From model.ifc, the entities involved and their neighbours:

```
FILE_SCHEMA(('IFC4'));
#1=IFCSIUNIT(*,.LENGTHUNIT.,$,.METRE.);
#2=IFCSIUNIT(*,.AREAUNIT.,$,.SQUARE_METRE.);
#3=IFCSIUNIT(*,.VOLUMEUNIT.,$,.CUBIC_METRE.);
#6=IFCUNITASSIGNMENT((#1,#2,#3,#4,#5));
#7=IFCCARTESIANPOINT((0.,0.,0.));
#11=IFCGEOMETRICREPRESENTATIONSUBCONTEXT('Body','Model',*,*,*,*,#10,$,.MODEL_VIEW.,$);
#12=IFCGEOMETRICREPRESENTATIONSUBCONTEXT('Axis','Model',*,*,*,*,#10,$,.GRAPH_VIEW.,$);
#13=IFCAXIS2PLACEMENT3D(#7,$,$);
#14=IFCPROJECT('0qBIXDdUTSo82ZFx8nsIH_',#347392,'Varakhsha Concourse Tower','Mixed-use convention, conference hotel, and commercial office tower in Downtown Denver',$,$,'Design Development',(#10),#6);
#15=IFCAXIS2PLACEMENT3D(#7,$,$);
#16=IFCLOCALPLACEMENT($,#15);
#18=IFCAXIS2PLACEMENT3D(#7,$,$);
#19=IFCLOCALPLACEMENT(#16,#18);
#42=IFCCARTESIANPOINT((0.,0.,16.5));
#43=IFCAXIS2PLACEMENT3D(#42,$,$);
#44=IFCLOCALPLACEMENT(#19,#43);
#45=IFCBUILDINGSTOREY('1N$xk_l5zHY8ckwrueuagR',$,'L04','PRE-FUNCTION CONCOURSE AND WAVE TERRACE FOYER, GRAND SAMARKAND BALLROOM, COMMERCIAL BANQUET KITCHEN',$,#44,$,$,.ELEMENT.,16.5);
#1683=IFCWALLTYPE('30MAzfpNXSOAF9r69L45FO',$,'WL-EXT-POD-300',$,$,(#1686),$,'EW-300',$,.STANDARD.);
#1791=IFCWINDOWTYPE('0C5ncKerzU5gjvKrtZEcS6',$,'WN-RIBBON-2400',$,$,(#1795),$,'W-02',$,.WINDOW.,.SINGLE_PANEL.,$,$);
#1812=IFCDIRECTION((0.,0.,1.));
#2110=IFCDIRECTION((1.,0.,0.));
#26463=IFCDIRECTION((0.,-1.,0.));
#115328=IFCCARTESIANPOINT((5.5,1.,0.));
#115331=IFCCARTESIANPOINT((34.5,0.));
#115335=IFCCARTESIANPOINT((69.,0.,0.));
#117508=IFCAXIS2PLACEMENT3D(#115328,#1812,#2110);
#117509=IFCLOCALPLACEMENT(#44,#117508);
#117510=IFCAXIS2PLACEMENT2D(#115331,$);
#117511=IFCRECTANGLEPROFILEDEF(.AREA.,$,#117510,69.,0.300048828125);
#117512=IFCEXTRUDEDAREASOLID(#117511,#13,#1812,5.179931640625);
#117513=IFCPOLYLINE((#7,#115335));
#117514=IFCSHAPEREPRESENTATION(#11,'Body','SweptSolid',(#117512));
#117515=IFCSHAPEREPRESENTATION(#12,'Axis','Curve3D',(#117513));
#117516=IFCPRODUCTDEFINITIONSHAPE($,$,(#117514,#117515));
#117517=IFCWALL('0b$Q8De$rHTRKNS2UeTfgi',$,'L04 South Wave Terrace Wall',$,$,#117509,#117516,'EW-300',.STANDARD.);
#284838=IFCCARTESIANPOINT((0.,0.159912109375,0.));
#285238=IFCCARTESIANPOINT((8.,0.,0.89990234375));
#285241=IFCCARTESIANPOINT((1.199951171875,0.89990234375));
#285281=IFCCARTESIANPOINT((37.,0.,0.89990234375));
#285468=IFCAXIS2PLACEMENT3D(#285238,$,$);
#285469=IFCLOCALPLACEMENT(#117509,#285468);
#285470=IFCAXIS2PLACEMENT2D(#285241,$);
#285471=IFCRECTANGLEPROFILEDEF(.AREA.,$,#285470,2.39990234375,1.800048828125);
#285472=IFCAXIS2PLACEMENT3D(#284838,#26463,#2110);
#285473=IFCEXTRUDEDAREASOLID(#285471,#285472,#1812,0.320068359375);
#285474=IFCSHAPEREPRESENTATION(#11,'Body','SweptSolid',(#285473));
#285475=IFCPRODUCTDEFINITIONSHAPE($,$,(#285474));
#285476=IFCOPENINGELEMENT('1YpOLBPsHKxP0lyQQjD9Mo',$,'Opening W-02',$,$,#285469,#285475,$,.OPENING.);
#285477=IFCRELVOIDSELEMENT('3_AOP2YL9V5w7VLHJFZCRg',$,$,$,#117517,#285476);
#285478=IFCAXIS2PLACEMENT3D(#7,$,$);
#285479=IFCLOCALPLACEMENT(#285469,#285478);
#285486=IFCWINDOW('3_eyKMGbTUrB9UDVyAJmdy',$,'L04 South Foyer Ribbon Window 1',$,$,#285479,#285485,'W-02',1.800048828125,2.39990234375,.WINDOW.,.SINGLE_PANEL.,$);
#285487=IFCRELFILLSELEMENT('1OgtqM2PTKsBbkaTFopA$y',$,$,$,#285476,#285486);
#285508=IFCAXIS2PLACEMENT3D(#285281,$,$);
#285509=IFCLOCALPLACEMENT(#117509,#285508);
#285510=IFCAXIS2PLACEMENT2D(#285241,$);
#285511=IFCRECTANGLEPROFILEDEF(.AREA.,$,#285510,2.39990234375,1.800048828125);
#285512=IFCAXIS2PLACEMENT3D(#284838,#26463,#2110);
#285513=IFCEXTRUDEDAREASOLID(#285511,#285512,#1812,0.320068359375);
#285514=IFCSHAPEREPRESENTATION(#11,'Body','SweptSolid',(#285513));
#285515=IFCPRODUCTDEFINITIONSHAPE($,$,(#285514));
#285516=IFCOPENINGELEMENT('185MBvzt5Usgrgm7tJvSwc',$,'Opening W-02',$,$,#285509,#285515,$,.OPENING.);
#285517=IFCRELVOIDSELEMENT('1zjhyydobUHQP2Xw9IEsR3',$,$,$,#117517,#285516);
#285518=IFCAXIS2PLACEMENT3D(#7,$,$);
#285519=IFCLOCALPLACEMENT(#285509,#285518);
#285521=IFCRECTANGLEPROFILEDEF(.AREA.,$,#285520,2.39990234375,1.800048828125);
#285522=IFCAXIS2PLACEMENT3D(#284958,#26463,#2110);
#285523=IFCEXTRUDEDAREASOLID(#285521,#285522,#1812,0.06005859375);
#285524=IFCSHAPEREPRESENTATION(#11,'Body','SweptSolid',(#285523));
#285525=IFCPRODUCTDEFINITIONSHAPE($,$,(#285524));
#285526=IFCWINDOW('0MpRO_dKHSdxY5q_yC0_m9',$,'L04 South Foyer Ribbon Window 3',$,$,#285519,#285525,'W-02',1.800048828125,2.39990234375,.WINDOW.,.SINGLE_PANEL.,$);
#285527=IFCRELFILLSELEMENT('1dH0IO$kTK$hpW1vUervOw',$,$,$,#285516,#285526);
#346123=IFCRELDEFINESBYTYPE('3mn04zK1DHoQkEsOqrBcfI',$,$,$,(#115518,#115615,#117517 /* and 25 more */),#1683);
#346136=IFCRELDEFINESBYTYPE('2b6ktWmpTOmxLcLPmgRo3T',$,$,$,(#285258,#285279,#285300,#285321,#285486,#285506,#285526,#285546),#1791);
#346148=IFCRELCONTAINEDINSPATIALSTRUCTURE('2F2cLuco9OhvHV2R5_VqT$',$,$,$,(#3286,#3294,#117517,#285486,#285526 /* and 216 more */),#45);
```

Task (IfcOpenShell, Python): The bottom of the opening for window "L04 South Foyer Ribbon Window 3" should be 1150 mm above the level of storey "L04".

```python
import numpy as np
import ifcopenshell
import ifcopenshell.api.geometry
import ifcopenshell.geom
import ifcopenshell.util.element
import ifcopenshell.util.placement
import ifcopenshell.util.shape
import ifcopenshell.util.unit

model = ifcopenshell.open("model.ifc")
unit_scale = ifcopenshell.util.unit.calculate_unit_scale(model)

window = model.by_guid("0MpRO_dKHSdxY5q_yC0_m9")
opening = window.FillsVoids[0].RelatingOpeningElement
storey = ifcopenshell.util.element.get_container(window, ifc_class="IfcBuildingStorey")
level = ifcopenshell.util.placement.get_local_placement(storey.ObjectPlacement)[2, 3]

# The opening's origin need not be at the sill, so measure its lowest point.
shape = ifcopenshell.geom.create_shape(ifcopenshell.geom.settings(), opening)
bottom = ifcopenshell.util.shape.get_shape_bottom_elevation(shape, shape.geometry) / unit_scale
dz = level + 1.15 - bottom

shift = np.array([0.0, 0.0, dz])
# The window is placed relative to its opening, so it follows when the opening moves.
matrix = ifcopenshell.util.placement.get_local_placement(opening.ObjectPlacement)
matrix[:3, 3] += shift
ifcopenshell.api.geometry.edit_object_placement(
    model, product=opening, matrix=matrix, is_si=False, should_transform_children=True
)

print(f"moved by {dz * unit_scale:+.3f} m")

model.write("model-out.ifc")
```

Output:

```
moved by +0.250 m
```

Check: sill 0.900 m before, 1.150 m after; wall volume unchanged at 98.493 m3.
